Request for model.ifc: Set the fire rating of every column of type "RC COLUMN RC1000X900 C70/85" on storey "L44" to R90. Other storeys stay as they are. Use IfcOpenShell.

First a look at what the model holds.

```python
import ifcopenshell
import ifcopenshell.util.element

model = ifcopenshell.open("model.ifc")
print(model.schema)
storey = next(s for s in model.by_type("IfcBuildingStorey") if s.Name == "L44")
columns = [e for e in ifcopenshell.util.element.get_decomposition(storey) if e.is_a("IfcColumn")]
seen = {}
for e in columns:
    element_type = ifcopenshell.util.element.get_type(e)
    key = (element_type.Name if element_type != e and element_type else None, ifcopenshell.util.element.get_pset(e, "Pset_ColumnCommon", "FireRating"))
    seen[key] = seen.get(key, 0) + 1
for (name, value), count in sorted(seen.items(), key=str):
    print(count, "x", name, "|", value)
```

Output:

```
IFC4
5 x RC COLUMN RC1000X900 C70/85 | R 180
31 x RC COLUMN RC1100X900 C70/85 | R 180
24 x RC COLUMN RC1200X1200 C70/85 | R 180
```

```python
import ifcopenshell
import ifcopenshell.api.pset
import ifcopenshell.util.element

model = ifcopenshell.open("model.ifc")

storey = next(s for s in model.by_type("IfcBuildingStorey") if s.Name == "L44")
columns = [e for e in ifcopenshell.util.element.get_decomposition(storey) if e.is_a("IfcColumn")]

count = 0
for e in columns:
    element_type = ifcopenshell.util.element.get_type(e)
    if element_type in (None, e) or element_type.Name != "RC COLUMN RC1000X900 C70/85":
        continue
    found = ifcopenshell.util.element.get_pset(e, "Pset_ColumnCommon", should_inherit=False)
    if found:
        pset = model.by_id(found["id"])
        if len(ifcopenshell.util.element.get_elements_by_pset(pset)) > 1:
            pset = ifcopenshell.api.pset.unshare_pset(model, products=[e], pset=pset)[0]
    else:
        pset = ifcopenshell.api.pset.add_pset(model, product=e, name="Pset_ColumnCommon")
    ifcopenshell.api.pset.edit_pset(model, pset=pset, properties={"FireRating": "R90"})
    count += 1

print(count, "columns updated")

model.write("model_edited.ifc")
```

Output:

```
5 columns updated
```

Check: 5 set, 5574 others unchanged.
